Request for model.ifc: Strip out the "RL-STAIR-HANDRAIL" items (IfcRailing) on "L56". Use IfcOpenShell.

First a look at what the model holds.

```python
import ifcopenshell
import ifcopenshell.util.element

model = ifcopenshell.open("model.ifc")
print(model.schema)
storey = next(s for s in model.by_type("IfcBuildingStorey") if s.Name == "L56")
railings = [e for e in ifcopenshell.util.element.get_decomposition(storey) if e.is_a("IfcRailing")]
seen = {}
for e in railings:
    element_type = ifcopenshell.util.element.get_type(e)
    name = element_type.Name if element_type not in (None, e) else None
    seen[name] = seen.get(name, 0) + 1
for name, count in sorted(seen.items(), key=str):
    print(count, "x", name)
```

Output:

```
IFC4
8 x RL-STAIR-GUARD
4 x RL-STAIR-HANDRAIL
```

```python
import ifcopenshell
import ifcopenshell.api.root
import ifcopenshell.util.element

model = ifcopenshell.open("model.ifc")

storey = next(s for s in model.by_type("IfcBuildingStorey") if s.Name == "L56")
railings = [e for e in ifcopenshell.util.element.get_decomposition(storey) if e.is_a("IfcRailing")]
targets = [e for e in railings if (t := ifcopenshell.util.element.get_type(e)) not in (None, e) and t.Name == "RL-STAIR-HANDRAIL"]

for e in targets:
    ifcopenshell.api.root.remove_product(model, product=e)
print(len(targets), "removed")

model.write("model_edited.ifc")
```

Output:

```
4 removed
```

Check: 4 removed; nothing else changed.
